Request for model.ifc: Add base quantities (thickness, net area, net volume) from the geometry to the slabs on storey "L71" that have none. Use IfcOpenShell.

First a look at what the model holds.

```python
import ifcopenshell
import ifcopenshell.util.element
import ifcopenshell.util.unit

model = ifcopenshell.open("model.ifc")
print(model.schema)
for unit_type in ("LENGTHUNIT", "AREAUNIT", "VOLUMEUNIT"):
    print(unit_type, ifcopenshell.util.unit.calculate_unit_scale(model, unit_type))
storey = next(s for s in model.by_type("IfcBuildingStorey") if s.Name == "L71")
slabs = [e for e in ifcopenshell.util.element.get_decomposition(storey) if e.is_a("IfcSlab")]
for e in sorted(slabs, key=lambda e: e.id()):
    print(e.id(), e.is_a(), e.Name, list(ifcopenshell.util.element.get_psets(e, qtos_only=True)), sep=" | ")
```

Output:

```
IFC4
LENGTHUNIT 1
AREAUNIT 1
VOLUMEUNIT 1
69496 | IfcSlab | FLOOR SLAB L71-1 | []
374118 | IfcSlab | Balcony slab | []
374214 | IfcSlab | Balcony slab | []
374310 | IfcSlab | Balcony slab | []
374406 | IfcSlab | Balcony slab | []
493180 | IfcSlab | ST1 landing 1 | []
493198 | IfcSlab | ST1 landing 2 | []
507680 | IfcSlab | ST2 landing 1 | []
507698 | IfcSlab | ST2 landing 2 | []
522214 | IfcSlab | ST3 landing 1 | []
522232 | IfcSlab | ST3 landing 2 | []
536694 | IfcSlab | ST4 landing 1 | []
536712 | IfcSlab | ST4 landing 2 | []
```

```python
import ifcopenshell
import ifcopenshell.api.pset
import ifcopenshell.geom
import ifcopenshell.util.element
import ifcopenshell.util.shape
import ifcopenshell.util.unit

model = ifcopenshell.open("model.ifc")
unit_scale = ifcopenshell.util.unit.calculate_unit_scale(model)
area_scale = ifcopenshell.util.unit.calculate_unit_scale(model, "AREAUNIT")
volume_scale = ifcopenshell.util.unit.calculate_unit_scale(model, "VOLUMEUNIT")
settings = ifcopenshell.geom.settings()

storey = next(s for s in model.by_type("IfcBuildingStorey") if s.Name == "L71")
slabs = [e for e in ifcopenshell.util.element.get_decomposition(storey) if e.is_a("IfcSlab")]

for e in sorted(slabs, key=lambda e: e.id()):
    if ifcopenshell.util.element.get_psets(e, qtos_only=True, should_inherit=False):
        continue
    # Geometry comes back in metres, in the element's own axes.
    shape = ifcopenshell.geom.create_shape(settings, e)
    values = {
        "Width": ifcopenshell.util.shape.get_z(shape.geometry) / unit_scale,
        "NetArea": ifcopenshell.util.shape.get_footprint_area(shape.geometry) / area_scale,
        "NetVolume": ifcopenshell.util.shape.get_volume(shape.geometry) / volume_scale,
    }
    qto = ifcopenshell.api.pset.add_qto(model, product=e, name="Qto_SlabBaseQuantities")
    ifcopenshell.api.pset.edit_qto(model, qto=qto, properties=values)
    print(e.id(), {k: round(v, 3) for k, v in values.items()})

model.write("model_updated.ifc")
```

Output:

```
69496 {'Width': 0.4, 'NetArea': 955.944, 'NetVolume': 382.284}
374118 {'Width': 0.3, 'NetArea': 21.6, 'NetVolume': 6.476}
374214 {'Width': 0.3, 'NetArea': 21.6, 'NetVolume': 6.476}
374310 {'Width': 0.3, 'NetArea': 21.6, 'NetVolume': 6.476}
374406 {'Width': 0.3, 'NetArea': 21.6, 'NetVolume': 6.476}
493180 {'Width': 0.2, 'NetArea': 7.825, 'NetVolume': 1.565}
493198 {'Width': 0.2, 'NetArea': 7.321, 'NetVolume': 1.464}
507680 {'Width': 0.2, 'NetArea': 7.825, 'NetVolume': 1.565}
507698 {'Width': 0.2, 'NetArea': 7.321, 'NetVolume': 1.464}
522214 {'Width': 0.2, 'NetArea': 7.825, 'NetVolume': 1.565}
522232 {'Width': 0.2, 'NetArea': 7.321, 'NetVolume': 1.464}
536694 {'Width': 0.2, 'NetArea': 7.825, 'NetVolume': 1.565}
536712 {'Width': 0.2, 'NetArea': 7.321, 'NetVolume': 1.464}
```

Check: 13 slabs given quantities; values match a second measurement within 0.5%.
